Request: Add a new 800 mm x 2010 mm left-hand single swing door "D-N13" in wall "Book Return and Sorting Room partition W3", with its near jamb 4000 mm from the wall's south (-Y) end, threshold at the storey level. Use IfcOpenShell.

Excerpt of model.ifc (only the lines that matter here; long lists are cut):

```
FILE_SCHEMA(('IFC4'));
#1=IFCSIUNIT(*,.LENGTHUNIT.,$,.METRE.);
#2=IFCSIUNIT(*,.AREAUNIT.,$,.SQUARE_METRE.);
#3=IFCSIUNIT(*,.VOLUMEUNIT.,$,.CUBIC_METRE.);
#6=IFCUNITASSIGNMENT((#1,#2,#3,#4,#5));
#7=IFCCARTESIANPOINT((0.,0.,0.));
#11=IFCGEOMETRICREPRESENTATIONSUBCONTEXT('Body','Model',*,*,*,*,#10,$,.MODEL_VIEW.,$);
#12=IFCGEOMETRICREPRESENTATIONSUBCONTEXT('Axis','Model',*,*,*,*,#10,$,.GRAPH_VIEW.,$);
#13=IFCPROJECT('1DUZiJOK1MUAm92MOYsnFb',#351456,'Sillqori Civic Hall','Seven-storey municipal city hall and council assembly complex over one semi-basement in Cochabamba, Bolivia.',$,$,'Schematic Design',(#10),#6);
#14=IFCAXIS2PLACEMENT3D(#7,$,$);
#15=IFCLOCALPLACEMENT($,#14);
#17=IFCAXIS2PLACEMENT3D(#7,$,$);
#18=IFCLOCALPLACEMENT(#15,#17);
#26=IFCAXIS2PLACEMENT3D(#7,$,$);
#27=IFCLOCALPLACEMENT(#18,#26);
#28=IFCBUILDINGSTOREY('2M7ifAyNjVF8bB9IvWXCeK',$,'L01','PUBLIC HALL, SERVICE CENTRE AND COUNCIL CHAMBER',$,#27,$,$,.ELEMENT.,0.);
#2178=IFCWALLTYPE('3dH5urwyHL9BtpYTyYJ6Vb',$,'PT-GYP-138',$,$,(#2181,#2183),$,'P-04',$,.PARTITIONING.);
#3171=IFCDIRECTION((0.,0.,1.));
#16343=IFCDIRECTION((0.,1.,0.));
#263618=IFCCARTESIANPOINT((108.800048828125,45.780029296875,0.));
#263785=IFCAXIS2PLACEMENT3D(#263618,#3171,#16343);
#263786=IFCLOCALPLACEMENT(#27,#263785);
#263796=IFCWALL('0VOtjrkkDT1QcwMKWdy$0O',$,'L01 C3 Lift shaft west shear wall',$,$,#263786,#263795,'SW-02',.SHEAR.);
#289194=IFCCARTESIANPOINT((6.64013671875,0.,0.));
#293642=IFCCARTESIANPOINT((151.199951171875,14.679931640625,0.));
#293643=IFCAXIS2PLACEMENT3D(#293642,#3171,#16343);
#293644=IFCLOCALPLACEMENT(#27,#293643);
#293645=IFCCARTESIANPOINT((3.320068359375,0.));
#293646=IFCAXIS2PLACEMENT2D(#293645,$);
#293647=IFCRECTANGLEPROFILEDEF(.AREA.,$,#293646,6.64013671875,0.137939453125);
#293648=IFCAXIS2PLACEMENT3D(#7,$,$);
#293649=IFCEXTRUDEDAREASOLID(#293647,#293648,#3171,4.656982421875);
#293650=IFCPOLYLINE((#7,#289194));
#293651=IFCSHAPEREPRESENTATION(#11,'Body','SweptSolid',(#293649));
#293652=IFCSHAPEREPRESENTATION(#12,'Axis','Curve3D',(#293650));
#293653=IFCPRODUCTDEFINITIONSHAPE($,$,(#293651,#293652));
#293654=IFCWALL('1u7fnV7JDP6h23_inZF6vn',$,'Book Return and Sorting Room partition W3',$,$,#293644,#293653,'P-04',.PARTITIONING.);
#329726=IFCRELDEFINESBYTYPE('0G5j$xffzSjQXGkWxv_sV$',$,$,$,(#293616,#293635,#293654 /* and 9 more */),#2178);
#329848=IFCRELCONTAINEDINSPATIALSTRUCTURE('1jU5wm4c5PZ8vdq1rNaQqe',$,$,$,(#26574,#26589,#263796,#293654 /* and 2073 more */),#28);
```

```python
import numpy as np
import ifcopenshell
import ifcopenshell.api.feature
import ifcopenshell.api.geometry
import ifcopenshell.api.root
import ifcopenshell.api.spatial
import ifcopenshell.geom
import ifcopenshell.util.element
import ifcopenshell.util.placement
import ifcopenshell.util.representation
import ifcopenshell.util.shape
import ifcopenshell.util.unit

model = ifcopenshell.open("model.ifc")
unit_scale = ifcopenshell.util.unit.calculate_unit_scale(model)
settings = ifcopenshell.geom.settings()


def volume(element):
    """Net volume in cubic metres, openings subtracted."""
    shape = ifcopenshell.geom.create_shape(settings, element)
    return ifcopenshell.util.shape.get_volume(shape.geometry)


wall = model.by_id(293654)
storey = ifcopenshell.util.element.get_container(wall, ifc_class="IfcBuildingStorey")
context = ifcopenshell.util.representation.get_context(model, "Model", "Body", "MODEL_VIEW")
before = volume(wall)

width, height, from_end, sill = 0.8, 2.01, 4, 0.0  # metres

# The wall runs along its own X axis, and the end named is its -X end.
wall_shape = ifcopenshell.geom.create_shape(settings, wall)
x, y, z = ifcopenshell.util.shape.get_vertices(wall_shape.geometry).T
start = x.min() + from_end
face, thickness = float(y.min()), float(y.max() - y.min())
wall_matrix = ifcopenshell.util.placement.get_local_placement(wall.ObjectPlacement)
level = ifcopenshell.util.placement.get_local_placement(storey.ObjectPlacement)[2, 3]


def in_wall(x, y):
    """Placement at x, y metres in the wall's axes, at sill height."""
    matrix = wall_matrix.copy()
    matrix[:, 3] = wall_matrix @ np.array([x / unit_scale, y / unit_scale, 0.0, 1.0])
    matrix[2, 3] = level + sill / unit_scale
    return matrix


# Opening: a box that overshoots both wall faces by 50 mm.
opening = ifcopenshell.api.root.create_entity(model, ifc_class="IfcOpeningElement", predefined_type="OPENING")
box = ifcopenshell.api.geometry.add_wall_representation(
    model, context=context, length=width, height=height, thickness=thickness + 0.1
)
ifcopenshell.api.geometry.assign_representation(model, product=opening, representation=box)
ifcopenshell.api.geometry.edit_object_placement(model, product=opening, matrix=in_wall(start, face - 0.05), is_si=False)
ifcopenshell.api.feature.add_feature(model, feature=opening, element=wall)

door = ifcopenshell.api.root.create_entity(model, ifc_class="IfcDoor", name="D-N13", predefined_type="DOOR")
door.OverallWidth, door.OverallHeight = width / unit_scale, height / unit_scale
door.OperationType = "SINGLE_SWING_LEFT"
body = ifcopenshell.api.geometry.add_door_representation(
    model,
    context=context,
    overall_width=door.OverallWidth,
    overall_height=door.OverallHeight,
    operation_type="SINGLE_SWING_LEFT",
    lining_properties={"LiningDepth": thickness / unit_scale, "ThresholdDepth": thickness / unit_scale},
)
ifcopenshell.api.geometry.assign_representation(model, product=door, representation=body)
ifcopenshell.api.spatial.assign_container(model, products=[door], relating_structure=storey)
ifcopenshell.api.feature.add_filling(model, opening=opening, element=door)

# The lining spans the wall, so the door starts at the wall face.
ifcopenshell.api.geometry.edit_object_placement(model, product=door, matrix=in_wall(start, face), is_si=False)

after = volume(wall)

print(f"wall volume {before:.3f} -> {after:.3f} m3")

model.write("model_edited.ifc")
```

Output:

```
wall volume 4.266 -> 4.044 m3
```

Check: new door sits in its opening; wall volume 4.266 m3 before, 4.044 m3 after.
